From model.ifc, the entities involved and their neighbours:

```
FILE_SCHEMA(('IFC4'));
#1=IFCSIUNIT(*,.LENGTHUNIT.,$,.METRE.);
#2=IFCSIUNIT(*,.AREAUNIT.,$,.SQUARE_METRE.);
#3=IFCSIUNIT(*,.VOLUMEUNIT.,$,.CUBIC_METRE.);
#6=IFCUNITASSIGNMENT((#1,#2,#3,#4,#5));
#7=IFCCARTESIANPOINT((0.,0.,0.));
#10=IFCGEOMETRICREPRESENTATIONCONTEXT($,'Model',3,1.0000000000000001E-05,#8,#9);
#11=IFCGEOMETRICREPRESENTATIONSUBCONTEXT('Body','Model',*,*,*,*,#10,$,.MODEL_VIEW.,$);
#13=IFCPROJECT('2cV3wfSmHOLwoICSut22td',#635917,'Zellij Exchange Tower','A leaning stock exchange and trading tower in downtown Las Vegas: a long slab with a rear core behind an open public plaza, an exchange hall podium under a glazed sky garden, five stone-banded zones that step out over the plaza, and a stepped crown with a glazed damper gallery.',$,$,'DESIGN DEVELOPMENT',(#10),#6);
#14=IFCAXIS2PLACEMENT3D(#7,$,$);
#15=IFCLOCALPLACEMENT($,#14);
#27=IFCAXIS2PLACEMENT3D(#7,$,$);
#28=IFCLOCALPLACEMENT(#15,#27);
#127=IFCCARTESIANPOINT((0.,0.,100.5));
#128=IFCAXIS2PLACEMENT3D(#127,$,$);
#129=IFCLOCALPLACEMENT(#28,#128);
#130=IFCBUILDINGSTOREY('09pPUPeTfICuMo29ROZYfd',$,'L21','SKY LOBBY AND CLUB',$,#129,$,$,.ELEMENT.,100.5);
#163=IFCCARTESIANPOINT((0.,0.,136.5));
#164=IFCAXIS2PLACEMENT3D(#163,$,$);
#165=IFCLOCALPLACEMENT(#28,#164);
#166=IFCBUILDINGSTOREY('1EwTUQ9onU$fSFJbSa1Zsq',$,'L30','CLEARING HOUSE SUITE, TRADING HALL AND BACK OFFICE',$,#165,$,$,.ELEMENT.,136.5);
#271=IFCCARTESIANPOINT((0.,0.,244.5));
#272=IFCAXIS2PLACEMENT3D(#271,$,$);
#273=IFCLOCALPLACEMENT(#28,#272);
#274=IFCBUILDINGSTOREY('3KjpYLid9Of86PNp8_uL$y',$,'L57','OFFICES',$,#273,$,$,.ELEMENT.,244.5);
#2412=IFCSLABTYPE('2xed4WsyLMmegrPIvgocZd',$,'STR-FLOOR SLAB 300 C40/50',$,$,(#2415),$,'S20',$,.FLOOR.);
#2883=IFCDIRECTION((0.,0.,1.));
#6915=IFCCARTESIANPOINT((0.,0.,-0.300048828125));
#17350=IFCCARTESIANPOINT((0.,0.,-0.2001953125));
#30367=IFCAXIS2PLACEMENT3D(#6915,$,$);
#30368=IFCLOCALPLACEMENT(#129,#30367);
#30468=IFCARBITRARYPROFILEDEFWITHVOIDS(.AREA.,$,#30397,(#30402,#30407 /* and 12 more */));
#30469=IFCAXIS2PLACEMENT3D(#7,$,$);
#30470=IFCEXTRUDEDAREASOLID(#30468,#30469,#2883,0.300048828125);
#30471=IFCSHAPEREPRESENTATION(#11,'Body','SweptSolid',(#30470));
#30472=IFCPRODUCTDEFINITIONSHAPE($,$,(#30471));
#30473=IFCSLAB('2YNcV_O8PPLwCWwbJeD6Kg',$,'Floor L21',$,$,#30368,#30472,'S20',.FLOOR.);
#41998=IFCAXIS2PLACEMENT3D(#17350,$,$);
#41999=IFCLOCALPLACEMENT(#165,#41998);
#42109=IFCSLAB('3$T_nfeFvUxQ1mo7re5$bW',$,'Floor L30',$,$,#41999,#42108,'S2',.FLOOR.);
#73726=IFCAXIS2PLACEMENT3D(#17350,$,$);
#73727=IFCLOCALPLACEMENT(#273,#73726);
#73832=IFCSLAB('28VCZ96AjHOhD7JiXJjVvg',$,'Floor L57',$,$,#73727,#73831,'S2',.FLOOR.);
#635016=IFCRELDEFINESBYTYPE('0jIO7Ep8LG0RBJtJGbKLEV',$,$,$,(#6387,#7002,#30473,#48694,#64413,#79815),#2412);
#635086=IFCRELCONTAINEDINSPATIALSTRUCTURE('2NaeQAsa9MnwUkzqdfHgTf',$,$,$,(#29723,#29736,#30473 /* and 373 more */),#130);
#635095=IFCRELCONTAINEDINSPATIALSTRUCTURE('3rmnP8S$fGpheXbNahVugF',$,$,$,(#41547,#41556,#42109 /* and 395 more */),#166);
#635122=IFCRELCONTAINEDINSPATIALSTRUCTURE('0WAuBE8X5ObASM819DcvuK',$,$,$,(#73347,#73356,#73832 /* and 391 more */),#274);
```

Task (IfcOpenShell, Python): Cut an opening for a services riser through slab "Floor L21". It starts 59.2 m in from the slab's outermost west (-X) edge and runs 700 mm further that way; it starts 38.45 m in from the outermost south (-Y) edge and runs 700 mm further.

```python
import numpy as np
import ifcopenshell
import ifcopenshell.api.feature
import ifcopenshell.api.geometry
import ifcopenshell.api.root
import ifcopenshell.geom
import ifcopenshell.util.placement
import ifcopenshell.util.representation
import ifcopenshell.util.shape
import ifcopenshell.util.unit

model = ifcopenshell.open("model.ifc")
unit_scale = ifcopenshell.util.unit.calculate_unit_scale(model)
settings = ifcopenshell.geom.settings()


def volume(element):
    """Net volume in cubic metres, openings subtracted."""
    shape = ifcopenshell.geom.create_shape(settings, element)
    return ifcopenshell.util.shape.get_volume(shape.geometry)


slab = model.by_id(30473)
before = volume(slab)

# Extent in the slab's own axes, in metres. The edges named are its -X and -Y sides.
slab_shape = ifcopenshell.geom.create_shape(settings, slab)
vertices = ifcopenshell.util.shape.get_vertices(slab_shape.geometry)
x_min, y_min, bottom = vertices.min(axis=0)
top = vertices[:, 2].max()

opening = ifcopenshell.api.root.create_entity(model, ifc_class="IfcOpeningElement", name="Services riser opening", predefined_type="OPENING")
context = ifcopenshell.util.representation.get_context(model, "Model", "Body", "MODEL_VIEW")
width, depth = 0.7, 0.7
outline = [(0.0, 0.0), (width, 0.0), (width, depth), (0.0, depth), (0.0, 0.0)]
# Overshoot both faces by 50 mm so the cut is clean.
shape = ifcopenshell.api.geometry.add_slab_representation(
    model, context=context, depth=top - bottom + 0.1, polyline=outline
)
ifcopenshell.api.geometry.assign_representation(model, product=opening, representation=shape)

matrix = ifcopenshell.util.placement.get_local_placement(slab.ObjectPlacement)
matrix[:, 3] = matrix @ np.append(np.array([x_min + 59.2, y_min + 38.45, bottom - 0.05]) / unit_scale, 1.0)
ifcopenshell.api.geometry.edit_object_placement(model, product=opening, matrix=matrix, is_si=False)
ifcopenshell.api.feature.add_feature(model, feature=opening, element=slab)

after = volume(slab)

print(f"slab volume {before:.3f} -> {after:.3f} m3")

model.write("model_v2.ifc")
```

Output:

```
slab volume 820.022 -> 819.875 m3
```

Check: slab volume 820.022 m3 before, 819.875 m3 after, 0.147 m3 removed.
